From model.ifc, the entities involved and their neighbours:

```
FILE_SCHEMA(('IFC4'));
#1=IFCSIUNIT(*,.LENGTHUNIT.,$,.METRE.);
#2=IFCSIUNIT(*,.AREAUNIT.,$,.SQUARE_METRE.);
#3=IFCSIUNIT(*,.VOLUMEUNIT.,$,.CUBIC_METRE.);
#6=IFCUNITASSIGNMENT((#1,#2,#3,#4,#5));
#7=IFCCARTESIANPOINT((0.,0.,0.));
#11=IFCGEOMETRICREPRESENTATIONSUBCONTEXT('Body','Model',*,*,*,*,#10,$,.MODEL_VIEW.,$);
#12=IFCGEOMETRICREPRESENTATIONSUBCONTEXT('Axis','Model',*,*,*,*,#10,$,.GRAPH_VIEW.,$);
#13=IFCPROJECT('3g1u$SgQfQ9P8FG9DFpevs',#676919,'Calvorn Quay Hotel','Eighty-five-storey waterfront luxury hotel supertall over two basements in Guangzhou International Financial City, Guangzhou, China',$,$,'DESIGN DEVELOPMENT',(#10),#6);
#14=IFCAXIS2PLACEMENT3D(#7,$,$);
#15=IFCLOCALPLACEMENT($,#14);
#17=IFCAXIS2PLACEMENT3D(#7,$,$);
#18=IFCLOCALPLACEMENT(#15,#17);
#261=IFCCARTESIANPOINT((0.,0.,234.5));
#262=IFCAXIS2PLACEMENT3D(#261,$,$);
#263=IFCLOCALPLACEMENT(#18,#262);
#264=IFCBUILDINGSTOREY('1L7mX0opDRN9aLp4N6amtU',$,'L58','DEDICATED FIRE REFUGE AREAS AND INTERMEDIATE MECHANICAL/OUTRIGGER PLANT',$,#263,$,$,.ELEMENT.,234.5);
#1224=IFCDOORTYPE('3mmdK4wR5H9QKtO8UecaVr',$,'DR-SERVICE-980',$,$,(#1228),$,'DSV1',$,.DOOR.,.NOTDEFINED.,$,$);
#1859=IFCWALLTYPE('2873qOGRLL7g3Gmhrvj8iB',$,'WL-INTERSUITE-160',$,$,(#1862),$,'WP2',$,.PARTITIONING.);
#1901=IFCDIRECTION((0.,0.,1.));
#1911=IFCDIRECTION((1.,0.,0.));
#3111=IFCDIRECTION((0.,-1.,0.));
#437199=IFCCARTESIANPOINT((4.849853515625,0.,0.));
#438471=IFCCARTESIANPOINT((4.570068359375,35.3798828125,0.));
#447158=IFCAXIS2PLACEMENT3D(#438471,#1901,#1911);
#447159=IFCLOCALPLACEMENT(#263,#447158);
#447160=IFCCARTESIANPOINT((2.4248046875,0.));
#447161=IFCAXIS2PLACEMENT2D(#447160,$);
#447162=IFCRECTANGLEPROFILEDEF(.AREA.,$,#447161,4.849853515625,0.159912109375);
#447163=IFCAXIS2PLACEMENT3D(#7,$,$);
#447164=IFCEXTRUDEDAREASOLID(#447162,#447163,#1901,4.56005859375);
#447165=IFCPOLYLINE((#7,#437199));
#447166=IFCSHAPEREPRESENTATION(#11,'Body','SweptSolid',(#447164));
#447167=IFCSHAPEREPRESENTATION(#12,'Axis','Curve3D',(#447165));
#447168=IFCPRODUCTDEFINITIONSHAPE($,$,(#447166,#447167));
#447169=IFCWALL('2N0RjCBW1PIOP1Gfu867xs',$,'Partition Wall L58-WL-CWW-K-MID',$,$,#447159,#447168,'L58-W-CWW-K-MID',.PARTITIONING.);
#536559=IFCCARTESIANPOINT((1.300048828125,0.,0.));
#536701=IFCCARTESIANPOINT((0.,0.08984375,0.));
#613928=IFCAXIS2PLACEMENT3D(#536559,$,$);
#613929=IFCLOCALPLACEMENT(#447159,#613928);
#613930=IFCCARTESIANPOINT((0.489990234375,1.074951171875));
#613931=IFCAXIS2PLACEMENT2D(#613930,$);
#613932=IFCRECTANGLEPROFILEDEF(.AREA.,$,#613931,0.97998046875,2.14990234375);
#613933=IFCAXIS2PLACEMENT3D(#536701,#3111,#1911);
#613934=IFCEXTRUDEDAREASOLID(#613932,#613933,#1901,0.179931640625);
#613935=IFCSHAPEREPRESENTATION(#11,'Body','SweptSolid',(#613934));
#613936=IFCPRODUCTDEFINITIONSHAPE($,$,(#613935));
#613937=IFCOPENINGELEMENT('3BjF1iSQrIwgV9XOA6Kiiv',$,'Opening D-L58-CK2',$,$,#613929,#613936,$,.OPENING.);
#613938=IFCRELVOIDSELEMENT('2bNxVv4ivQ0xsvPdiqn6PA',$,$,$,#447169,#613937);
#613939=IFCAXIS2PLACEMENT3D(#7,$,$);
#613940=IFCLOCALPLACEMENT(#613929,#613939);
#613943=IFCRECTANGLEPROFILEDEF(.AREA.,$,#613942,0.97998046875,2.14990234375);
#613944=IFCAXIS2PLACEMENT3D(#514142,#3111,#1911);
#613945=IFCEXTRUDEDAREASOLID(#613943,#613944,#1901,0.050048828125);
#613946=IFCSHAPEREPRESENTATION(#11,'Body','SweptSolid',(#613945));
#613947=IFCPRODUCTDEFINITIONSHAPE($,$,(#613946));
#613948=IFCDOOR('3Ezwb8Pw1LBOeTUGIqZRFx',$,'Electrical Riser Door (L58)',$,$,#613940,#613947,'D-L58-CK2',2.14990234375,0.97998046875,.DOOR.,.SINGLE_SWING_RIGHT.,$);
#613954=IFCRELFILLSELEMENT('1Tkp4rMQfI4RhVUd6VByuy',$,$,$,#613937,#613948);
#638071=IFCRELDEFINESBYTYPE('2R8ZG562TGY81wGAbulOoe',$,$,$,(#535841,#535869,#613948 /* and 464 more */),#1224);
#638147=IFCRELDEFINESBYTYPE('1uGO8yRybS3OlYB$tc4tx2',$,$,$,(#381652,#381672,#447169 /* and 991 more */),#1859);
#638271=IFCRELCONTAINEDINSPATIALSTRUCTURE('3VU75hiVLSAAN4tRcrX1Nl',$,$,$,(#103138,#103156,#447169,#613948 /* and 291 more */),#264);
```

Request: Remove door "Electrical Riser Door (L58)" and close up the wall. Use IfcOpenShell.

```python
import ifcopenshell
import ifcopenshell.api.feature
import ifcopenshell.api.root
import ifcopenshell.geom
import ifcopenshell.util.shape

model = ifcopenshell.open("model.ifc")
settings = ifcopenshell.geom.settings()


def volume(element):
    """Net volume in cubic metres, openings subtracted."""
    shape = ifcopenshell.geom.create_shape(settings, element)
    return ifcopenshell.util.shape.get_volume(shape.geometry)


door = model.by_guid("3Ezwb8Pw1LBOeTUGIqZRFx")
opening = door.FillsVoids[0].RelatingOpeningElement
wall = opening.VoidsElements[0].RelatingBuildingElement
before = volume(wall)

ifcopenshell.api.root.remove_product(model, product=door)
ifcopenshell.api.feature.remove_feature(model, feature=opening)

after = volume(wall)

print(f"wall volume {before:.3f} -> {after:.3f} m3")

model.write("model_edited.ifc")
```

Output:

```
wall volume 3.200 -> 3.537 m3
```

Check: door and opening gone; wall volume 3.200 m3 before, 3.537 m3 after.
